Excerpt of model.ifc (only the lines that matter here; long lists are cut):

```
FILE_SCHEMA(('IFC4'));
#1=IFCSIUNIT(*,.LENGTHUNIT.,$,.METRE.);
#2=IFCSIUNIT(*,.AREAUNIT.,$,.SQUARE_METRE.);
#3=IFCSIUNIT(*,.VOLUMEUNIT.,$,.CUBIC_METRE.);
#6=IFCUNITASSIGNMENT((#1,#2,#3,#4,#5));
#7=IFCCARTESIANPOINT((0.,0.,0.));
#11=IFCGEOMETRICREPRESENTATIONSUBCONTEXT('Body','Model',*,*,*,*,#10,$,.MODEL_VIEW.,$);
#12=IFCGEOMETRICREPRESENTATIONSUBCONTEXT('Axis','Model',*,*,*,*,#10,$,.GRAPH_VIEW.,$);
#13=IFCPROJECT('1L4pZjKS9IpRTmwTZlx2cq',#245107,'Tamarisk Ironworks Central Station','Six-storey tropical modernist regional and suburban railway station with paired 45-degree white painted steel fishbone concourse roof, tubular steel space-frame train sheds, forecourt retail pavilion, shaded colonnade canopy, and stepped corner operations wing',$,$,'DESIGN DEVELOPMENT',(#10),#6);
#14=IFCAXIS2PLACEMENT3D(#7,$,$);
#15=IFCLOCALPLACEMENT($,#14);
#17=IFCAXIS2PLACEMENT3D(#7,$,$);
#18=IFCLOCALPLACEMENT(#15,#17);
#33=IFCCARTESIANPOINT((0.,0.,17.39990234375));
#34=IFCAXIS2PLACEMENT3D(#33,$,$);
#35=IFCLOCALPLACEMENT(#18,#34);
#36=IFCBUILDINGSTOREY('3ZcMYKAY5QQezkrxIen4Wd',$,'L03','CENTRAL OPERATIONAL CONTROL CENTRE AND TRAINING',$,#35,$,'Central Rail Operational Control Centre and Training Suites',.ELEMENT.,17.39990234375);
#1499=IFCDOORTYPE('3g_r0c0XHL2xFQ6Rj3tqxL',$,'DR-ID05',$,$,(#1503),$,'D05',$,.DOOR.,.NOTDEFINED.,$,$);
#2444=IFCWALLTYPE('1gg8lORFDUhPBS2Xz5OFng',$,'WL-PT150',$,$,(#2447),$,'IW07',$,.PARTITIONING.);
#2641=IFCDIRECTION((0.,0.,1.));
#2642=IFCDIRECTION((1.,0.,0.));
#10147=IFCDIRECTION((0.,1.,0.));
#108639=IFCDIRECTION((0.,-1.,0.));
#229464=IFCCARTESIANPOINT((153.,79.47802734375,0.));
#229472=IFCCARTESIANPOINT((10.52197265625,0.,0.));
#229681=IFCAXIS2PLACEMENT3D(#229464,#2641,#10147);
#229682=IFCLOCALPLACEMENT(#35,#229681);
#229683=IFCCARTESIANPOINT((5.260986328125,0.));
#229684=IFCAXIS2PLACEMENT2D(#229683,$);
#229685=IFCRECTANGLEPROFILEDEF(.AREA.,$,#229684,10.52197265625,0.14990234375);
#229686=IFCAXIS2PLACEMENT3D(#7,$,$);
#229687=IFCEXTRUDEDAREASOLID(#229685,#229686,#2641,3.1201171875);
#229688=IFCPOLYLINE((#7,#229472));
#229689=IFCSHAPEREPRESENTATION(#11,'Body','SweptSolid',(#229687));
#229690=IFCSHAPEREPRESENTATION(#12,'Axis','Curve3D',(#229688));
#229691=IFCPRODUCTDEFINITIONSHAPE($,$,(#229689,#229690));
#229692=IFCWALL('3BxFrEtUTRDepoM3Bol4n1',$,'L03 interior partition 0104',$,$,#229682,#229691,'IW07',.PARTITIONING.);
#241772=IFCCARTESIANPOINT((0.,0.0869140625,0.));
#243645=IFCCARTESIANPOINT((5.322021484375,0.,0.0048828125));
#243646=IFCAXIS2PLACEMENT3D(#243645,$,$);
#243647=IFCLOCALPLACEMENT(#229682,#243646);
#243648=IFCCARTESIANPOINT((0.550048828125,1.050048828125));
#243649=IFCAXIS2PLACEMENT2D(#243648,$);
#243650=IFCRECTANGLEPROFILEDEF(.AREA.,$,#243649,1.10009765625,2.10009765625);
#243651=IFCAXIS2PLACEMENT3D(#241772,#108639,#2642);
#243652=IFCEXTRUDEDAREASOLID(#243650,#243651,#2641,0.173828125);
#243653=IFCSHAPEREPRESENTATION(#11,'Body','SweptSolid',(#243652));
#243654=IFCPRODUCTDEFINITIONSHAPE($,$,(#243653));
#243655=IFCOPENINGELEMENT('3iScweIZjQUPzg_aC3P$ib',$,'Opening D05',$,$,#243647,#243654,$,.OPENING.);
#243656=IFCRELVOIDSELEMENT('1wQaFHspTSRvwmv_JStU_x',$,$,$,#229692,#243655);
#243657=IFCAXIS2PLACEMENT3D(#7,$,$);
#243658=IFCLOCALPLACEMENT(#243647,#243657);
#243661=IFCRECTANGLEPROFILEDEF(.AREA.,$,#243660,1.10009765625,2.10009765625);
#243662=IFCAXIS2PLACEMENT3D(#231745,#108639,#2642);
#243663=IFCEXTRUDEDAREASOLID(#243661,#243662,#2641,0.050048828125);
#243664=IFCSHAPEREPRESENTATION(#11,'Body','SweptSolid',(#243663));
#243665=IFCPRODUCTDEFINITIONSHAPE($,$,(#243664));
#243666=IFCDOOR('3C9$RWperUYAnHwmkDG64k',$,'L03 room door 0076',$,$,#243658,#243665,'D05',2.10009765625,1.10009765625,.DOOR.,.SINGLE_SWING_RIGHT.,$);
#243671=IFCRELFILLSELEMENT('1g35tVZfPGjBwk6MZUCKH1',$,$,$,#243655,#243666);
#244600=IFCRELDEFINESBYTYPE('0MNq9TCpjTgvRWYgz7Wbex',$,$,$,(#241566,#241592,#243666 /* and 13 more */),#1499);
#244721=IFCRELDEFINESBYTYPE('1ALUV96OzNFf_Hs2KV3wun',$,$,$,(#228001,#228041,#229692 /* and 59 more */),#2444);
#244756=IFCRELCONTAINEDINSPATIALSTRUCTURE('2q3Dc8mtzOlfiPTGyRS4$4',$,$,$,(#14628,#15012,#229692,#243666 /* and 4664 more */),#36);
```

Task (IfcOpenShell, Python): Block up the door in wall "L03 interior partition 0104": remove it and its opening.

```python
import ifcopenshell
import ifcopenshell.api.feature
import ifcopenshell.api.root
import ifcopenshell.geom
import ifcopenshell.util.shape

model = ifcopenshell.open("model.ifc")
settings = ifcopenshell.geom.settings()


def volume(element):
    """Net volume in cubic metres, openings subtracted."""
    shape = ifcopenshell.geom.create_shape(settings, element)
    return ifcopenshell.util.shape.get_volume(shape.geometry)


door = model.by_guid("3C9$RWperUYAnHwmkDG64k")
opening = door.FillsVoids[0].RelatingOpeningElement
wall = opening.VoidsElements[0].RelatingBuildingElement
before = volume(wall)

ifcopenshell.api.root.remove_product(model, product=door)
ifcopenshell.api.feature.remove_feature(model, feature=opening)

after = volume(wall)

print(f"wall volume {before:.3f} -> {after:.3f} m3")

model.write("model_v2.ifc")
```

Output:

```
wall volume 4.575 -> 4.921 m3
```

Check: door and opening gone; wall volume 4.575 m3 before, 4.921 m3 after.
